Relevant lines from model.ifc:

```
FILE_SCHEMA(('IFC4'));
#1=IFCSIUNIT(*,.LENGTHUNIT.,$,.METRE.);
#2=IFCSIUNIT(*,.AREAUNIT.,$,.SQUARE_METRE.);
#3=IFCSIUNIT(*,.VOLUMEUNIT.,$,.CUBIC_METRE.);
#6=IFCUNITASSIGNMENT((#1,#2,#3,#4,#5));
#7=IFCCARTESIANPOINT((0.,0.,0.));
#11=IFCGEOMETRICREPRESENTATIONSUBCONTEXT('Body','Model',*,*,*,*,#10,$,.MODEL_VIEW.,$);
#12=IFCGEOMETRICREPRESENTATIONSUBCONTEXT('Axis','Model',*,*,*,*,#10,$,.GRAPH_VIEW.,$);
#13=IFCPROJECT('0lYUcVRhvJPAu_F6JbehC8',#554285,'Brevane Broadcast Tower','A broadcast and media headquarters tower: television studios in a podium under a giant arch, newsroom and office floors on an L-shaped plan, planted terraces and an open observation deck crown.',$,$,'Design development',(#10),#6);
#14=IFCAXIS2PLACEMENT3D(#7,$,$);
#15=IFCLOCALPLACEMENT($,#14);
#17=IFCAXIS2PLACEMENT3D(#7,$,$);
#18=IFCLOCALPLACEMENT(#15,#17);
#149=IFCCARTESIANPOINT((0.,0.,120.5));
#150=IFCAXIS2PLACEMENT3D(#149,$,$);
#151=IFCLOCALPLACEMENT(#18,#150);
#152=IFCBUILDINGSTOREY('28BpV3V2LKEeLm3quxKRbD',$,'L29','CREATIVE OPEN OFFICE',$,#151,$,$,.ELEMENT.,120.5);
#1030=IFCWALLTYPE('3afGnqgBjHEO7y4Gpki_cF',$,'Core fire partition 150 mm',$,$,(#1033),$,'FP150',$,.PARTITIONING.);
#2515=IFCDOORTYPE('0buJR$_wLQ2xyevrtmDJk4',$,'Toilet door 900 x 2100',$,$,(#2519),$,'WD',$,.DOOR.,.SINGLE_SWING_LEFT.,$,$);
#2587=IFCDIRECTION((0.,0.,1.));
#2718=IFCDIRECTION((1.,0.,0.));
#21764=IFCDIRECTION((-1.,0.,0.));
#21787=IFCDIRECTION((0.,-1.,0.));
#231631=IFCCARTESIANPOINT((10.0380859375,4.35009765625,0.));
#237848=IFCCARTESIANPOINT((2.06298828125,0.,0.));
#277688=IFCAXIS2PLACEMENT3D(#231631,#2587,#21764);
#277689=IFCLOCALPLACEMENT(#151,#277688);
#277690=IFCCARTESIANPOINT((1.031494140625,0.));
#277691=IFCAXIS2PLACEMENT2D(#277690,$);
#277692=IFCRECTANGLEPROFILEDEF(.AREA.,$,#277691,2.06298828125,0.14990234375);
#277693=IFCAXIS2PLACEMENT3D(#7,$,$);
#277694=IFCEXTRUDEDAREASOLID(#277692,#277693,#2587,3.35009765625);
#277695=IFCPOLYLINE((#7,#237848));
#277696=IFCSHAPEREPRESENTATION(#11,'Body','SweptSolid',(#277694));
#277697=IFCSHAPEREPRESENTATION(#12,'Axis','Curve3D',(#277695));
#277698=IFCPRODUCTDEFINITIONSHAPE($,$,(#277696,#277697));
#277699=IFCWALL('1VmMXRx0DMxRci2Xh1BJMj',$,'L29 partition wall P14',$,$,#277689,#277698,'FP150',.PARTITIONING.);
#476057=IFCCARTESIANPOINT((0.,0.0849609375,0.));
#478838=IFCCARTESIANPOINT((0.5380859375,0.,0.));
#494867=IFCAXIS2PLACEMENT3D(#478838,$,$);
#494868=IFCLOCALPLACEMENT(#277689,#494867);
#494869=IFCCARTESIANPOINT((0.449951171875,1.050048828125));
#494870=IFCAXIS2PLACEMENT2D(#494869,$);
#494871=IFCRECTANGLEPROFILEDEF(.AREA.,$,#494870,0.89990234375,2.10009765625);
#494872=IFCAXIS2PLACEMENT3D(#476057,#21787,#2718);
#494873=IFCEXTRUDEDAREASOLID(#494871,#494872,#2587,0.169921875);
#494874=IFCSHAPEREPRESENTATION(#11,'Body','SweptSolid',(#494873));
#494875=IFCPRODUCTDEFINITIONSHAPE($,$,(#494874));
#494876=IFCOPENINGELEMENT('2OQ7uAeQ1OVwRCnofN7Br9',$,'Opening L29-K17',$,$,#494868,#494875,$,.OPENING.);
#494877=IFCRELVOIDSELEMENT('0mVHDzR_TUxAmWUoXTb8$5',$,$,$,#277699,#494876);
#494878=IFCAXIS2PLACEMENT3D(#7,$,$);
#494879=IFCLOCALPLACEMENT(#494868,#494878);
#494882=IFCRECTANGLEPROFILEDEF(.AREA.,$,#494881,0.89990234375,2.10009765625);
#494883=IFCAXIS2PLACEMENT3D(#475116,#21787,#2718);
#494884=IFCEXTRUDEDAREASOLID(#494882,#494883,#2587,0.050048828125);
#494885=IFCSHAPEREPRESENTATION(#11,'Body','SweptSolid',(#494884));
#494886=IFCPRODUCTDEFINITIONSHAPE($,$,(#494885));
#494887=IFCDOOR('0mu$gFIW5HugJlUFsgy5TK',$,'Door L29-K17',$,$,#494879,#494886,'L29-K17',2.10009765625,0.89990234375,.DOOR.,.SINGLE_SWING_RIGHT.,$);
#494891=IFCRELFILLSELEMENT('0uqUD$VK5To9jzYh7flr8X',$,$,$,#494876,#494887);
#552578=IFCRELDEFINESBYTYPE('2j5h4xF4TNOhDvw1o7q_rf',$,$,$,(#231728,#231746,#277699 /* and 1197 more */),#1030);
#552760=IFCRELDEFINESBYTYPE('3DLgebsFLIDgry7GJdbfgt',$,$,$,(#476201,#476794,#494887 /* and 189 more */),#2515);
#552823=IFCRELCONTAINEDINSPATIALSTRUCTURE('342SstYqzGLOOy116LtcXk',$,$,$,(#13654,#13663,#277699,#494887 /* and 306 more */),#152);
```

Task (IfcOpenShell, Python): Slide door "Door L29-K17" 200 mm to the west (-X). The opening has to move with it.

```python
import ifcopenshell
import ifcopenshell.api.geometry
import ifcopenshell.util.placement
import ifcopenshell.util.unit

model = ifcopenshell.open("model.ifc")
unit_scale = ifcopenshell.util.unit.calculate_unit_scale(model)

door = model.by_guid("0mu$gFIW5HugJlUFsgy5TK")
opening = door.FillsVoids[0].RelatingOpeningElement
wall = opening.VoidsElements[0].RelatingBuildingElement

wall_matrix = ifcopenshell.util.placement.get_local_placement(wall.ObjectPlacement)
shift = wall_matrix[:3, 0] * 0.2 / unit_scale
before = ifcopenshell.util.placement.get_local_placement(door.ObjectPlacement)[:3, 3].copy()

# The door is placed relative to its opening, so it follows when the opening moves.
matrix = ifcopenshell.util.placement.get_local_placement(opening.ObjectPlacement)
matrix[:3, 3] += shift
ifcopenshell.api.geometry.edit_object_placement(
    model, product=opening, matrix=matrix, is_si=False, should_transform_children=True
)

after = ifcopenshell.util.placement.get_local_placement(door.ObjectPlacement)[:3, 3]
print("door moved by", (after - before).round(3) + 0.0)

model.write("model-out.ifc")
```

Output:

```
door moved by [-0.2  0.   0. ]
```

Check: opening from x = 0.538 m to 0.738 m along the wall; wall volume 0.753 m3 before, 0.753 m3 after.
